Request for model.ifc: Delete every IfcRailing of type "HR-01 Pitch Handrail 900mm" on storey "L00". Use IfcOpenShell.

First a look at what the model holds.

```python
import ifcopenshell
import ifcopenshell.util.element

model = ifcopenshell.open("model.ifc")
print(model.schema)
storey = next(s for s in model.by_type("IfcBuildingStorey") if s.Name == "L00")
railings = [e for e in ifcopenshell.util.element.get_decomposition(storey) if e.is_a("IfcRailing")]
seen = {}
for e in railings:
    element_type = ifcopenshell.util.element.get_type(e)
    name = element_type.Name if element_type not in (None, e) else None
    seen[name] = seen.get(name, 0) + 1
for name, count in sorted(seen.items(), key=str):
    print(count, "x", name)
```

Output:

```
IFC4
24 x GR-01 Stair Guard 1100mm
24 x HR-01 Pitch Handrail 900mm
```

```python
import ifcopenshell
import ifcopenshell.api.root
import ifcopenshell.util.element

model = ifcopenshell.open("model.ifc")

storey = next(s for s in model.by_type("IfcBuildingStorey") if s.Name == "L00")
railings = [e for e in ifcopenshell.util.element.get_decomposition(storey) if e.is_a("IfcRailing")]
targets = [e for e in railings if (t := ifcopenshell.util.element.get_type(e)) not in (None, e) and t.Name == "HR-01 Pitch Handrail 900mm"]

for e in targets:
    ifcopenshell.api.root.remove_product(model, product=e)
print(len(targets), "removed")

model.write("model_v2.ifc")
```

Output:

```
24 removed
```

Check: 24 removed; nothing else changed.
